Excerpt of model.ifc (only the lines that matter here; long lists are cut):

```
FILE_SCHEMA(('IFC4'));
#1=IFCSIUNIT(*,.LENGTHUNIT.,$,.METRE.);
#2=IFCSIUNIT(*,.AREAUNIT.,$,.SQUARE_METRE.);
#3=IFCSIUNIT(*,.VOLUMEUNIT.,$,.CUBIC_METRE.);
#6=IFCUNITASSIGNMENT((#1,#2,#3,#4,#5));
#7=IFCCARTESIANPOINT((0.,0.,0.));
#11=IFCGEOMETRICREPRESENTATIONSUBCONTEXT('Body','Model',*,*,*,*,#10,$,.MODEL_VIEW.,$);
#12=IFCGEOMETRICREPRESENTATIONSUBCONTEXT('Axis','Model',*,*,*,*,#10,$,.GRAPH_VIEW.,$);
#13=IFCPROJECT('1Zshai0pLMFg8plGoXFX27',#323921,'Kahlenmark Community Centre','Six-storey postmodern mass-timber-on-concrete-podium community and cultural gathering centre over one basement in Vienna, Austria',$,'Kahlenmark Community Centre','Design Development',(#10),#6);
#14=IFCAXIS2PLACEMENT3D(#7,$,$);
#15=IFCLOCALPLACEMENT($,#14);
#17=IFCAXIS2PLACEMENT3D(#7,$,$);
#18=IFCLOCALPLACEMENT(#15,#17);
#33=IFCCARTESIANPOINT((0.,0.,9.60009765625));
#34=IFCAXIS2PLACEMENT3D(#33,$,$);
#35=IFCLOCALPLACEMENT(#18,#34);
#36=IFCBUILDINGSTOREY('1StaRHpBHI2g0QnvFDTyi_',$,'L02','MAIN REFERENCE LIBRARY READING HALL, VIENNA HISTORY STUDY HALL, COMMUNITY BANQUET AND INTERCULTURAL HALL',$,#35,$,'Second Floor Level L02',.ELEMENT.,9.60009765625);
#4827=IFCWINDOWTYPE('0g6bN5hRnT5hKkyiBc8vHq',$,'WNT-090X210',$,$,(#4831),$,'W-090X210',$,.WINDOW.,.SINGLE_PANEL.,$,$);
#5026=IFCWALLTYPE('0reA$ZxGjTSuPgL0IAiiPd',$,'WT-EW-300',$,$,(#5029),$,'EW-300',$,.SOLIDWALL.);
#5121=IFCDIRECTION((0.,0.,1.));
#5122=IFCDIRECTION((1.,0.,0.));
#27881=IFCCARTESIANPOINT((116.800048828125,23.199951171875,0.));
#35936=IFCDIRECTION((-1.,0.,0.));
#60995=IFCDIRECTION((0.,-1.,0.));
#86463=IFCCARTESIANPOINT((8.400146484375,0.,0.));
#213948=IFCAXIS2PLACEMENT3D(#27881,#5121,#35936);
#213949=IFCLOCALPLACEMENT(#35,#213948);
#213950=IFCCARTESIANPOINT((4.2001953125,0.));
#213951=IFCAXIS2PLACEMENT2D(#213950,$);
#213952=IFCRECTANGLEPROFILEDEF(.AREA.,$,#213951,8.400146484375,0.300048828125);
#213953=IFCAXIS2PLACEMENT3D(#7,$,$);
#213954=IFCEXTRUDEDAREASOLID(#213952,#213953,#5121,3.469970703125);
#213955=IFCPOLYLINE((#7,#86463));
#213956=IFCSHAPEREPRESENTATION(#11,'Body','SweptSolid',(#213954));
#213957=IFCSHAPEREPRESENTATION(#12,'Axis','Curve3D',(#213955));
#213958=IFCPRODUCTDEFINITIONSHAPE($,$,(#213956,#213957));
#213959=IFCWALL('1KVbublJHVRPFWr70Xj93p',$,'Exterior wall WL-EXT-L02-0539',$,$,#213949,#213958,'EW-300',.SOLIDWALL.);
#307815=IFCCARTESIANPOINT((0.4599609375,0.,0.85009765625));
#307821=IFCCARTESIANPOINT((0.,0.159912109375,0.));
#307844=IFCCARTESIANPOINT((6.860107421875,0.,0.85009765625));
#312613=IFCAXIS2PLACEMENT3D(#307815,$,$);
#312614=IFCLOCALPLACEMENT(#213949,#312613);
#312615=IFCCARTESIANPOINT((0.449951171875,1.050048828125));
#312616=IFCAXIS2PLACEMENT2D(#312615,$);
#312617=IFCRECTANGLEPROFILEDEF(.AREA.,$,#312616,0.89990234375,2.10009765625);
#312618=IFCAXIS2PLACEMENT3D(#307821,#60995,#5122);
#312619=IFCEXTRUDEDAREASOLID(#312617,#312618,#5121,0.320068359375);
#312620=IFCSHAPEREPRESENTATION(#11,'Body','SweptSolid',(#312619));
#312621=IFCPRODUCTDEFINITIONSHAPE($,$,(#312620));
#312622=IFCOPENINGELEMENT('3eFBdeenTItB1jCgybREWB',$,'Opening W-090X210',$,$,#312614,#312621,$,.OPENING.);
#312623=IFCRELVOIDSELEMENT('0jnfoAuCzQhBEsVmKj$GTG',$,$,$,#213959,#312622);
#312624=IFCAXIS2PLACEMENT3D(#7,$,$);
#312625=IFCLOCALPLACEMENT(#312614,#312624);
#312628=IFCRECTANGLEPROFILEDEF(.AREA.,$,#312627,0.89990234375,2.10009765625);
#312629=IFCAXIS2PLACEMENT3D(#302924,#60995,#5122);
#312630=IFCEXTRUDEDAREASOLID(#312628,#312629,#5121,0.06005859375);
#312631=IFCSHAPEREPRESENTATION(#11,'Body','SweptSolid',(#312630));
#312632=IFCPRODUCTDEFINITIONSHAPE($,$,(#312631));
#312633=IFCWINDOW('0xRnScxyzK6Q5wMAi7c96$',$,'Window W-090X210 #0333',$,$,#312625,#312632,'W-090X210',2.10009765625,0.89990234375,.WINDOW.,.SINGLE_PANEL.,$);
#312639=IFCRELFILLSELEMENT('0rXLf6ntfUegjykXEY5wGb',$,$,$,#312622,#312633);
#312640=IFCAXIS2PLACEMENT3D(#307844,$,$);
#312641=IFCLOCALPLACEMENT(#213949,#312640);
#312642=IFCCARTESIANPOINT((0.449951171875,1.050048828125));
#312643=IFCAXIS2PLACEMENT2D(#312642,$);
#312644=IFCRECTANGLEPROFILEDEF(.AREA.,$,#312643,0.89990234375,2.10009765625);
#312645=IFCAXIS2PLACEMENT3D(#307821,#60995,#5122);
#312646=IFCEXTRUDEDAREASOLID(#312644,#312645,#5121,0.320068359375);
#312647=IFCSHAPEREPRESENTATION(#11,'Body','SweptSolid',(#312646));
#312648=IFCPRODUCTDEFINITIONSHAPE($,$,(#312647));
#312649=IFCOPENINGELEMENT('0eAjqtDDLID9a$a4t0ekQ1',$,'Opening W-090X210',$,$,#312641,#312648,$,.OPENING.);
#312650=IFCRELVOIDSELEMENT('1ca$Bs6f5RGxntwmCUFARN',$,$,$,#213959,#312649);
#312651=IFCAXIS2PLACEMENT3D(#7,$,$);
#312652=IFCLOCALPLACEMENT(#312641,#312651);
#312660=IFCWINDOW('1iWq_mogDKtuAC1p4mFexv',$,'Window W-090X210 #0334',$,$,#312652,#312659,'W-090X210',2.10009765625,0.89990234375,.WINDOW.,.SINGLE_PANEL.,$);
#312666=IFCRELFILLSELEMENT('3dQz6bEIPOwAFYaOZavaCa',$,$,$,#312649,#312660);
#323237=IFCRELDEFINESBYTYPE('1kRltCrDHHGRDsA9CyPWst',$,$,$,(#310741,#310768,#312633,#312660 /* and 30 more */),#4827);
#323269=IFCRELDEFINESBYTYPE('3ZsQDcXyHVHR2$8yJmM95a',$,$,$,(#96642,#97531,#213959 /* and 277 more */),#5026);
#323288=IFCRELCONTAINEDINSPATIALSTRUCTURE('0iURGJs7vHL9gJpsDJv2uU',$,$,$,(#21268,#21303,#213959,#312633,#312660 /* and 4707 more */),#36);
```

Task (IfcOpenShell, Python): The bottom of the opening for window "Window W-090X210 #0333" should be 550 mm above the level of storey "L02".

```python
import numpy as np
import ifcopenshell
import ifcopenshell.api.geometry
import ifcopenshell.geom
import ifcopenshell.util.element
import ifcopenshell.util.placement
import ifcopenshell.util.shape
import ifcopenshell.util.unit

model = ifcopenshell.open("model.ifc")
unit_scale = ifcopenshell.util.unit.calculate_unit_scale(model)

window = model.by_guid("0xRnScxyzK6Q5wMAi7c96$")
opening = window.FillsVoids[0].RelatingOpeningElement
storey = ifcopenshell.util.element.get_container(window, ifc_class="IfcBuildingStorey")
level = ifcopenshell.util.placement.get_local_placement(storey.ObjectPlacement)[2, 3]

# The opening's origin need not be at the sill, so measure its lowest point.
shape = ifcopenshell.geom.create_shape(ifcopenshell.geom.settings(), opening)
bottom = ifcopenshell.util.shape.get_shape_bottom_elevation(shape, shape.geometry) / unit_scale
dz = level + 0.55 / unit_scale - bottom

shift = np.array([0.0, 0.0, dz])
# The window is placed relative to its opening, so it follows when the opening moves.
matrix = ifcopenshell.util.placement.get_local_placement(opening.ObjectPlacement)
matrix[:3, 3] += shift
ifcopenshell.api.geometry.edit_object_placement(
    model, product=opening, matrix=matrix, is_si=False, should_transform_children=True
)

print(f"moved by {dz * unit_scale:+.3f} m")

model.write("model-out.ifc")
```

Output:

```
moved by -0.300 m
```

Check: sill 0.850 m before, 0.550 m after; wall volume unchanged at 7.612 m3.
